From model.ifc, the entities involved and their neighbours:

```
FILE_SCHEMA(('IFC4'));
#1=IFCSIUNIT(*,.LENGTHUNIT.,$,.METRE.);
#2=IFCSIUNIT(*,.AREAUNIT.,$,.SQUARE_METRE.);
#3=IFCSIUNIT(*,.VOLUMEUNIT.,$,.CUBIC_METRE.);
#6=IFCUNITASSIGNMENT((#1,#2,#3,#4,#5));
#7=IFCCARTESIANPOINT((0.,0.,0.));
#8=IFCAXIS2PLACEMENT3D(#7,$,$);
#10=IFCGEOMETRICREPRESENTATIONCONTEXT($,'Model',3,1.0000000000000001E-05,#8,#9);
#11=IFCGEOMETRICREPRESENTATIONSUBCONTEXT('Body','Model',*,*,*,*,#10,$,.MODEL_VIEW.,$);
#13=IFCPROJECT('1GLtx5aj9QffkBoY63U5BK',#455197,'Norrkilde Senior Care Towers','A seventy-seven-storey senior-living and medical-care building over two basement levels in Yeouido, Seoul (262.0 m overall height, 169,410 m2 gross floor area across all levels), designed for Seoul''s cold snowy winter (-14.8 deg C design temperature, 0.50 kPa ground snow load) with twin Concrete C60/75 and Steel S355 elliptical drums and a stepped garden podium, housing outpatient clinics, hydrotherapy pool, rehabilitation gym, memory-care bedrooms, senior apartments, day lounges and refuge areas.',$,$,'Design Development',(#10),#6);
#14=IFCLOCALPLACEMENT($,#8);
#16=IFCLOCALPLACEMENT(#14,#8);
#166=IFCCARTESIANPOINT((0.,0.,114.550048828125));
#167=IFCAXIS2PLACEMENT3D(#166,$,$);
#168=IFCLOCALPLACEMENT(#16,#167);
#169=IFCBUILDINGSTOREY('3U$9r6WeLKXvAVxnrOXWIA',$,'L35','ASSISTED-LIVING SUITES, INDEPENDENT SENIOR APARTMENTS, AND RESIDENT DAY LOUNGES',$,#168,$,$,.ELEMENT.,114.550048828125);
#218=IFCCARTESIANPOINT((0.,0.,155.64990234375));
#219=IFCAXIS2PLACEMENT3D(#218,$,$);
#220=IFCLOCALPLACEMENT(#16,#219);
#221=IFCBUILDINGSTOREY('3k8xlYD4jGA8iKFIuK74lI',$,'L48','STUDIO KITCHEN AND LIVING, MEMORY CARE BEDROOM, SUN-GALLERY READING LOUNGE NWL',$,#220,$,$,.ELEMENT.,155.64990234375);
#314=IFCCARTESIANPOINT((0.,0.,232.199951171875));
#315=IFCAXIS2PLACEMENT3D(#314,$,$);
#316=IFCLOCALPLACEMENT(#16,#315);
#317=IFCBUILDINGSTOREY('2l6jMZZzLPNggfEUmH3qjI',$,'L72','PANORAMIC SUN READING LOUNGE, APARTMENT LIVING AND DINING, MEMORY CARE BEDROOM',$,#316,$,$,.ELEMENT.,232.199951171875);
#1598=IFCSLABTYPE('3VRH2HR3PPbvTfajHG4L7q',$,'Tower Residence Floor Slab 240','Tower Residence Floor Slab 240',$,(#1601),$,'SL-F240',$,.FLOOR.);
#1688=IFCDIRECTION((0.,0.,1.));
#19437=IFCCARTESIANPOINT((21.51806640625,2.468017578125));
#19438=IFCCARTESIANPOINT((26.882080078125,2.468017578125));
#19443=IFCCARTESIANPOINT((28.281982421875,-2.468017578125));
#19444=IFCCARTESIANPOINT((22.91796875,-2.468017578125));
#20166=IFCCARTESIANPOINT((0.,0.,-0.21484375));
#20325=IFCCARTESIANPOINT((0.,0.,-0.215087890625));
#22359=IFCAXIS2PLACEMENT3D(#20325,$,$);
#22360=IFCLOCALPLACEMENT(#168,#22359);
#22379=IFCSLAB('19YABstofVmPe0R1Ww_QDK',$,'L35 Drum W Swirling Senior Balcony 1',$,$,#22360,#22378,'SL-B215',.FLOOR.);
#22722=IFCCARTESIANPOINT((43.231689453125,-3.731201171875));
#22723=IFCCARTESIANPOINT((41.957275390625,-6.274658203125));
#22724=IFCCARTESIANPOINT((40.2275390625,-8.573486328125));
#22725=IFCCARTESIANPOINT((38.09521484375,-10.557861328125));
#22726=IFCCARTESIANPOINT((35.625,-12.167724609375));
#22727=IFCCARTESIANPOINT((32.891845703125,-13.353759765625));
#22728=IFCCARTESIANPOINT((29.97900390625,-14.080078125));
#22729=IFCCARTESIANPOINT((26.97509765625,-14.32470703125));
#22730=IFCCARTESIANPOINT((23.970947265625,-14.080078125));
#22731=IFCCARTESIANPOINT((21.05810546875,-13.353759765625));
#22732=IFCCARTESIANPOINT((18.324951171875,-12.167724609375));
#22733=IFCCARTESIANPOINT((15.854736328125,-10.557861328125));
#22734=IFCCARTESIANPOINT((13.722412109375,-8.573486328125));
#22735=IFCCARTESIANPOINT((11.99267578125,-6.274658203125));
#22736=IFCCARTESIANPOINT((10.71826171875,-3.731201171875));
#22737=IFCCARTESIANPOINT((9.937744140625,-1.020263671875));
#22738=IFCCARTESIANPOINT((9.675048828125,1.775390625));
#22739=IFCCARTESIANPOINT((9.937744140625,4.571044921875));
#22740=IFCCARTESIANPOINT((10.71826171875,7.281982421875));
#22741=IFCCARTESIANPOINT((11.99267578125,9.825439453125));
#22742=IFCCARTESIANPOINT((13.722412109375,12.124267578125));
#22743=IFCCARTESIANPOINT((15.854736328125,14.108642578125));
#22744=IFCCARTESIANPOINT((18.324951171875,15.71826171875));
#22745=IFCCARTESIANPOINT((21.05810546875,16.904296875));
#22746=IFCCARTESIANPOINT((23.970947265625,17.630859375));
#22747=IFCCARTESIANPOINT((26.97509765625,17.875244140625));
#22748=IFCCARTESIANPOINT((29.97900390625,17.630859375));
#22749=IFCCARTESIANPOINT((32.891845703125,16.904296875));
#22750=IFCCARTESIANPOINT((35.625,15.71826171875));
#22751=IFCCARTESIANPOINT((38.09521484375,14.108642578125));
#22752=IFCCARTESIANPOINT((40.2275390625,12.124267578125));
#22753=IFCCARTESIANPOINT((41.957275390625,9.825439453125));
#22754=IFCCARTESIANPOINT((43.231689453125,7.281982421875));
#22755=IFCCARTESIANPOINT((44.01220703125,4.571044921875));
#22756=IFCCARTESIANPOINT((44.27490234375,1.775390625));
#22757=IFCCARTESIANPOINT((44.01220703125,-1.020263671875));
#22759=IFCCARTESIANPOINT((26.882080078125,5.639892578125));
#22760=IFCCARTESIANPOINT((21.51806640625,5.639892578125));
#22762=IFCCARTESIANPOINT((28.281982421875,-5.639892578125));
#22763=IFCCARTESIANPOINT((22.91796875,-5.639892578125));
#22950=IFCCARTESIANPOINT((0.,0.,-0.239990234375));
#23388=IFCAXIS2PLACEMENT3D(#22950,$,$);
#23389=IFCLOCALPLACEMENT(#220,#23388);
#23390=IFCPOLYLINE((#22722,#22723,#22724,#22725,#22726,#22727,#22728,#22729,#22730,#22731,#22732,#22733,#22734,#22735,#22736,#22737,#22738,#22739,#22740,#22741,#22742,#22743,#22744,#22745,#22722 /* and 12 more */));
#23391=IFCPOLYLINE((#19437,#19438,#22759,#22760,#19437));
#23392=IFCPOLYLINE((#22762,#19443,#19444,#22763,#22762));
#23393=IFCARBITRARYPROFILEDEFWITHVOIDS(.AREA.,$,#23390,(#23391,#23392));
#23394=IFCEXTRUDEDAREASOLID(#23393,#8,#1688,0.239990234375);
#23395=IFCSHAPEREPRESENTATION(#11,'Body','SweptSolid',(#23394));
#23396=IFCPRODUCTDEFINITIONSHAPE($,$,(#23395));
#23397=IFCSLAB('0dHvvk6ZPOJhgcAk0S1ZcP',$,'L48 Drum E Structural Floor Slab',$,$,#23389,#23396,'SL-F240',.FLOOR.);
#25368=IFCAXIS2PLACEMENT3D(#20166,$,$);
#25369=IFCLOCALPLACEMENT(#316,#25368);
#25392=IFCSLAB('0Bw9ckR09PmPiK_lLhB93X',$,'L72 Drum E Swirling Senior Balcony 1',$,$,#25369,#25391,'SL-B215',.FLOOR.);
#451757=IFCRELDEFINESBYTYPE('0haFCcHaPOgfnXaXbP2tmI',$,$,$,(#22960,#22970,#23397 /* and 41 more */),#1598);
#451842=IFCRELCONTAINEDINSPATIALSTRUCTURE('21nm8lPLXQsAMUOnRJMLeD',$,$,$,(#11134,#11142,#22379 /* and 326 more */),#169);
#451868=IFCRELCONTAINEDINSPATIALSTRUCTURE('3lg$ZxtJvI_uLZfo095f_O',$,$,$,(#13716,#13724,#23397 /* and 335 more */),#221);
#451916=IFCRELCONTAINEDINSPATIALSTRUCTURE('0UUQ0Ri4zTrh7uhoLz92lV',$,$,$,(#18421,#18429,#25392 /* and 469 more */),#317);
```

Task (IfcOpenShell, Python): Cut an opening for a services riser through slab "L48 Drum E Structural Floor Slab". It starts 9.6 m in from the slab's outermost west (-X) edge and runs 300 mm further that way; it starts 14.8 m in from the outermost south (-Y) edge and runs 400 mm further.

```python
import numpy as np
import ifcopenshell
import ifcopenshell.api.feature
import ifcopenshell.api.geometry
import ifcopenshell.api.root
import ifcopenshell.geom
import ifcopenshell.util.placement
import ifcopenshell.util.representation
import ifcopenshell.util.shape
import ifcopenshell.util.unit

model = ifcopenshell.open("model.ifc")
unit_scale = ifcopenshell.util.unit.calculate_unit_scale(model)
settings = ifcopenshell.geom.settings()


def volume(element):
    """Net volume in cubic metres, openings subtracted."""
    shape = ifcopenshell.geom.create_shape(settings, element)
    return ifcopenshell.util.shape.get_volume(shape.geometry)


slab = model.by_guid("0dHvvk6ZPOJhgcAk0S1ZcP")
before = volume(slab)

# Extent in the slab's own axes, in metres. The edges named are its -X and -Y sides.
slab_shape = ifcopenshell.geom.create_shape(settings, slab)
vertices = ifcopenshell.util.shape.get_vertices(slab_shape.geometry)
x_min, y_min, bottom = vertices.min(axis=0)
top = vertices[:, 2].max()

opening = ifcopenshell.api.root.create_entity(model, ifc_class="IfcOpeningElement", name="Services riser opening", predefined_type="OPENING")
context = ifcopenshell.util.representation.get_context(model, "Model", "Body", "MODEL_VIEW")
width, depth = 0.3, 0.4
outline = [(0.0, 0.0), (width, 0.0), (width, depth), (0.0, depth), (0.0, 0.0)]
# Overshoot both faces by 50 mm so the cut is clean.
shape = ifcopenshell.api.geometry.add_slab_representation(
    model, context=context, depth=top - bottom + 0.1, polyline=outline
)
ifcopenshell.api.geometry.assign_representation(model, product=opening, representation=shape)

matrix = ifcopenshell.util.placement.get_local_placement(slab.ObjectPlacement)
matrix[:, 3] = matrix @ np.append(np.array([x_min + 9.6, y_min + 14.8, bottom - 0.05]) / unit_scale, 1.0)
ifcopenshell.api.geometry.edit_object_placement(model, product=opening, matrix=matrix, is_si=False)
ifcopenshell.api.feature.add_feature(model, feature=opening, element=slab)

after = volume(slab)

print(f"slab volume {before:.3f} -> {after:.3f} m3")

model.write("model_v2.ifc")
```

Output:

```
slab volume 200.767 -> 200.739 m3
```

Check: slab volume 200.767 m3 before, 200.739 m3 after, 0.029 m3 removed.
